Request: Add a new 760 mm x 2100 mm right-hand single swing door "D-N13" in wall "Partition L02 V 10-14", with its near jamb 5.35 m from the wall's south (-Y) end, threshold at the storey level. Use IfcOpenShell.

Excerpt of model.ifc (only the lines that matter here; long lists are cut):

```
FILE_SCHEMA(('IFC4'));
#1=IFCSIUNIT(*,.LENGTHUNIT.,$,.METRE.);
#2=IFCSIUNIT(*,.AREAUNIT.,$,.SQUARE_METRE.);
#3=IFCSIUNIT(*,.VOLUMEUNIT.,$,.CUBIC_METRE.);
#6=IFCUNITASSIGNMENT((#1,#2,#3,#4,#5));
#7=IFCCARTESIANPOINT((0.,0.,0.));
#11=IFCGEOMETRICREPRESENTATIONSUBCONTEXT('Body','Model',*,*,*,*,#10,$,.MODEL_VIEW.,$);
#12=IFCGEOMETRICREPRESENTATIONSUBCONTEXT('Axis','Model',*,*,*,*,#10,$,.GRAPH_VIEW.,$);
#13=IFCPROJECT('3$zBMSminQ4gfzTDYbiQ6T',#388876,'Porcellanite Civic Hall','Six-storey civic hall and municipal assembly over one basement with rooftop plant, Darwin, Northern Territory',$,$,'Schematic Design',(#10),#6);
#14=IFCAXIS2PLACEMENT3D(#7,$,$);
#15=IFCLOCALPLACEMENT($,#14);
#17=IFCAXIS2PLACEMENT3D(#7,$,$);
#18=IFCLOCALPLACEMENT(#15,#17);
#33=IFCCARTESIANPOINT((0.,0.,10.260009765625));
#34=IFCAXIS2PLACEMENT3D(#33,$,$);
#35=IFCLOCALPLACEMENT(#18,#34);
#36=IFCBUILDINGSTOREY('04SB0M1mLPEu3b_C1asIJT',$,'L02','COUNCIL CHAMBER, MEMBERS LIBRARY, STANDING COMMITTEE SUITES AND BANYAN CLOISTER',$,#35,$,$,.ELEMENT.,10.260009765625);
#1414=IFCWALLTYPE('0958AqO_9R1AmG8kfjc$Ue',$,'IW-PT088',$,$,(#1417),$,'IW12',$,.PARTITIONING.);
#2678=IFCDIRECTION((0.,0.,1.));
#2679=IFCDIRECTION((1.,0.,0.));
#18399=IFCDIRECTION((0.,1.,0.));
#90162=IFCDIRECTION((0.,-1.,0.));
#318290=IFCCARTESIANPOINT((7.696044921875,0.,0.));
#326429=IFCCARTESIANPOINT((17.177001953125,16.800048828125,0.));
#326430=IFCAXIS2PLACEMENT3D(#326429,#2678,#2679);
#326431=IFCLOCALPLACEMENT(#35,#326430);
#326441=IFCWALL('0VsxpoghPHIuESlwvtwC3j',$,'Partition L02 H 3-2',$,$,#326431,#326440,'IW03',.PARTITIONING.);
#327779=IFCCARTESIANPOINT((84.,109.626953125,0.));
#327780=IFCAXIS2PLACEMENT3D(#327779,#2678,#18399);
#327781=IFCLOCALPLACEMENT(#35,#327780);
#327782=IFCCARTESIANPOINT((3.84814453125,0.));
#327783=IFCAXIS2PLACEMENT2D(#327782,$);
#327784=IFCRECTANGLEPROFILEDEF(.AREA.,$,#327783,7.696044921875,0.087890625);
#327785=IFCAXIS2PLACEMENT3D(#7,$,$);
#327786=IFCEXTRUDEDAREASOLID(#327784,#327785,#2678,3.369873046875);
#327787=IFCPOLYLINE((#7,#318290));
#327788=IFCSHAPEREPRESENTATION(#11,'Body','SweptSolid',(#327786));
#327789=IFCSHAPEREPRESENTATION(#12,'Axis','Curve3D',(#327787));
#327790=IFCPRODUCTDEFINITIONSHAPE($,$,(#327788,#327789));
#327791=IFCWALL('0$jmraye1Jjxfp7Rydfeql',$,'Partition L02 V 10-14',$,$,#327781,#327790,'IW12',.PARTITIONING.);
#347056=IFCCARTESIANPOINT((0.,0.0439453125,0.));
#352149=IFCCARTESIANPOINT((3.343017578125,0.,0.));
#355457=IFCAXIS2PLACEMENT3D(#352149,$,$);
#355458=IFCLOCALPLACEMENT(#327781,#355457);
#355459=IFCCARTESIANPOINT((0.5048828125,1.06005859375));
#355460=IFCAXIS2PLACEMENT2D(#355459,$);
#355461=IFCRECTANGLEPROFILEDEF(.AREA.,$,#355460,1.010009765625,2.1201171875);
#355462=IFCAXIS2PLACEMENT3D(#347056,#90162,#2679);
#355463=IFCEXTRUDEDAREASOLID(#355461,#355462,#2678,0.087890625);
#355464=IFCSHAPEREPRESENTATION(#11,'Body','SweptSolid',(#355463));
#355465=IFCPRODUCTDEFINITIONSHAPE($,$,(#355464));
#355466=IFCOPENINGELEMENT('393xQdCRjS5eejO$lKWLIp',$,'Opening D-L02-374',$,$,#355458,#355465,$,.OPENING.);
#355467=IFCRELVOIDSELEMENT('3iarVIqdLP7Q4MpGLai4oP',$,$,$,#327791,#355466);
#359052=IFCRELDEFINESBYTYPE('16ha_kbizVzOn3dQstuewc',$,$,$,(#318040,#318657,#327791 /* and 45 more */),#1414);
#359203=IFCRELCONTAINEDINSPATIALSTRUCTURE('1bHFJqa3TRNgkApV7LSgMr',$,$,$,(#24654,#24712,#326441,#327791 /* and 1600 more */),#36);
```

```python
import numpy as np
import ifcopenshell
import ifcopenshell.api.feature
import ifcopenshell.api.geometry
import ifcopenshell.api.root
import ifcopenshell.api.spatial
import ifcopenshell.geom
import ifcopenshell.util.element
import ifcopenshell.util.placement
import ifcopenshell.util.representation
import ifcopenshell.util.shape
import ifcopenshell.util.unit

model = ifcopenshell.open("model.ifc")
unit_scale = ifcopenshell.util.unit.calculate_unit_scale(model)
settings = ifcopenshell.geom.settings()


def volume(element):
    """Net volume in cubic metres, openings subtracted."""
    shape = ifcopenshell.geom.create_shape(settings, element)
    return ifcopenshell.util.shape.get_volume(shape.geometry)


wall = model.by_guid("0$jmraye1Jjxfp7Rydfeql")
storey = ifcopenshell.util.element.get_container(wall, ifc_class="IfcBuildingStorey")
context = ifcopenshell.util.representation.get_context(model, "Model", "Body", "MODEL_VIEW")
before = volume(wall)

width, height, from_end, sill = 0.76, 2.1, 5.35, 0.0  # metres

# The wall runs along its own X axis, and the end named is its -X end.
wall_shape = ifcopenshell.geom.create_shape(settings, wall)
x, y, z = ifcopenshell.util.shape.get_vertices(wall_shape.geometry).T
start = x.min() + from_end
face, thickness = float(y.min()), float(y.max() - y.min())
wall_matrix = ifcopenshell.util.placement.get_local_placement(wall.ObjectPlacement)
level = ifcopenshell.util.placement.get_local_placement(storey.ObjectPlacement)[2, 3]


def in_wall(x, y):
    """Placement at x, y metres in the wall's axes, at sill height."""
    matrix = wall_matrix.copy()
    matrix[:, 3] = wall_matrix @ np.array([x / unit_scale, y / unit_scale, 0.0, 1.0])
    matrix[2, 3] = level + sill / unit_scale
    return matrix


# Opening: a box that overshoots both wall faces by 50 mm.
opening = ifcopenshell.api.root.create_entity(model, ifc_class="IfcOpeningElement", predefined_type="OPENING")
box = ifcopenshell.api.geometry.add_wall_representation(
    model, context=context, length=width, height=height, thickness=thickness + 0.1
)
ifcopenshell.api.geometry.assign_representation(model, product=opening, representation=box)
ifcopenshell.api.geometry.edit_object_placement(model, product=opening, matrix=in_wall(start, face - 0.05), is_si=False)
ifcopenshell.api.feature.add_feature(model, feature=opening, element=wall)

door = ifcopenshell.api.root.create_entity(model, ifc_class="IfcDoor", name="D-N13", predefined_type="DOOR")
door.OverallWidth, door.OverallHeight = width / unit_scale, height / unit_scale
door.OperationType = "SINGLE_SWING_RIGHT"
body = ifcopenshell.api.geometry.add_door_representation(
    model,
    context=context,
    overall_width=door.OverallWidth,
    overall_height=door.OverallHeight,
    operation_type="SINGLE_SWING_RIGHT",
    lining_properties={"LiningDepth": thickness / unit_scale, "ThresholdDepth": thickness / unit_scale},
)
ifcopenshell.api.geometry.assign_representation(model, product=door, representation=body)
ifcopenshell.api.spatial.assign_container(model, products=[door], relating_structure=storey)
ifcopenshell.api.feature.add_filling(model, opening=opening, element=door)

# The lining spans the wall, so the door starts at the wall face.
ifcopenshell.api.geometry.edit_object_placement(model, product=door, matrix=in_wall(start, face), is_si=False)

after = volume(wall)

print(f"wall volume {before:.3f} -> {after:.3f} m3")

model.write("model-out.ifc")
```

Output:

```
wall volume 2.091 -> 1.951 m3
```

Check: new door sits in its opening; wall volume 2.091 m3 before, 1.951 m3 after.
